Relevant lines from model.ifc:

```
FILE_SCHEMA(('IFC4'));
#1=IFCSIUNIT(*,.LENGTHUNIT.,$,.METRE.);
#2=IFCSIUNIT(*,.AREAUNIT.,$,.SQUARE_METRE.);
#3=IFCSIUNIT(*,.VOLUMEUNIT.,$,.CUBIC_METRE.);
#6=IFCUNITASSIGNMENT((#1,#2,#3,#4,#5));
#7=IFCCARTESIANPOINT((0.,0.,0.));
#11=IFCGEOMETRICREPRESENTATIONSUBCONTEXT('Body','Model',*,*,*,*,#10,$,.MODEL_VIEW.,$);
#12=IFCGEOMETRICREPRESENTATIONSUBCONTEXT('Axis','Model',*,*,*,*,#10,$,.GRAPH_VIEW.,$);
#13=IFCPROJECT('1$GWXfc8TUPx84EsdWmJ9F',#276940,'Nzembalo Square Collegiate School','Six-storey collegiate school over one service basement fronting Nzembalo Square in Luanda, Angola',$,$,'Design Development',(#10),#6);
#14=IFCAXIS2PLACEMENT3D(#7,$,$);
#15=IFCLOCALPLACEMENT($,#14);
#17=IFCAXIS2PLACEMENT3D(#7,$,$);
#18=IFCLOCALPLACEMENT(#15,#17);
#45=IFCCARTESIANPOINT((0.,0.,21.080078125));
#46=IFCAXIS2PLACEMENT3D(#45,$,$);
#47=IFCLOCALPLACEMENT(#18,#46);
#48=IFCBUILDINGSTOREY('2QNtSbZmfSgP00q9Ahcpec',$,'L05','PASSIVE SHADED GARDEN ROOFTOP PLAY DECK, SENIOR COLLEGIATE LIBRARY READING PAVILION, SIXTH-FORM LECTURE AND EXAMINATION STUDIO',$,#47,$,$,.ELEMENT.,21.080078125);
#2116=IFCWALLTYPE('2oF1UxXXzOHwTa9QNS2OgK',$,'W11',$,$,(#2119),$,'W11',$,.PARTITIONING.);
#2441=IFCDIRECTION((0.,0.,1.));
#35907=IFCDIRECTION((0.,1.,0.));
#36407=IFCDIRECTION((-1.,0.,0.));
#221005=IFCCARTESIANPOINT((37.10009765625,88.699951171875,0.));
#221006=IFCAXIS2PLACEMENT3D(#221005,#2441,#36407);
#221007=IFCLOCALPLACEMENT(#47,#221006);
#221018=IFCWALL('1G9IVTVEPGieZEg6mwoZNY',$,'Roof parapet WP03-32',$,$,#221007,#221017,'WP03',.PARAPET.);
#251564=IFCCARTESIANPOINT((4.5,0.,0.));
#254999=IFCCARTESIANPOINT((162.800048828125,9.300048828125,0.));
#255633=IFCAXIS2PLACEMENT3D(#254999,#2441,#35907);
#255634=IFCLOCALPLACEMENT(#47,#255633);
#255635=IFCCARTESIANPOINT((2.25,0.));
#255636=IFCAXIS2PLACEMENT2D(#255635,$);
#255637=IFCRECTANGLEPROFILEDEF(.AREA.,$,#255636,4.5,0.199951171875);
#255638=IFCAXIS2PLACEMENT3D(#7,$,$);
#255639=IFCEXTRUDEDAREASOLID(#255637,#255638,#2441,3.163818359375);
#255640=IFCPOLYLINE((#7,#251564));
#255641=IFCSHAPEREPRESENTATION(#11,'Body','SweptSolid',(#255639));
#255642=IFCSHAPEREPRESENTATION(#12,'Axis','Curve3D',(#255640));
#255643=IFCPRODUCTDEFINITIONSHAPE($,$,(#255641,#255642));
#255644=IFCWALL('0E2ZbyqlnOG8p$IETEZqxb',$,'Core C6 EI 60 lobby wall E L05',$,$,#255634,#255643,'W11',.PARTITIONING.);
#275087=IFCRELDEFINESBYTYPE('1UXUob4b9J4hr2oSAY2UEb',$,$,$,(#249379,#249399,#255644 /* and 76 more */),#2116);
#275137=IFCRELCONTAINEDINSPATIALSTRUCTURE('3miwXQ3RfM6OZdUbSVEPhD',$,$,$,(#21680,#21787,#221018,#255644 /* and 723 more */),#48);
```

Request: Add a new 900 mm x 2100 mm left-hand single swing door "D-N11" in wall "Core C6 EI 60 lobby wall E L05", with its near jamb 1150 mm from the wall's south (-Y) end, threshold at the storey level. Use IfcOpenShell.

```python
import numpy as np
import ifcopenshell
import ifcopenshell.api.feature
import ifcopenshell.api.geometry
import ifcopenshell.api.root
import ifcopenshell.api.spatial
import ifcopenshell.geom
import ifcopenshell.util.element
import ifcopenshell.util.placement
import ifcopenshell.util.representation
import ifcopenshell.util.shape
import ifcopenshell.util.unit

model = ifcopenshell.open("model.ifc")
unit_scale = ifcopenshell.util.unit.calculate_unit_scale(model)
settings = ifcopenshell.geom.settings()


def volume(element):
    """Net volume in cubic metres, openings subtracted."""
    shape = ifcopenshell.geom.create_shape(settings, element)
    return ifcopenshell.util.shape.get_volume(shape.geometry)


wall = model.by_id(255644)
storey = ifcopenshell.util.element.get_container(wall, ifc_class="IfcBuildingStorey")
context = ifcopenshell.util.representation.get_context(model, "Model", "Body", "MODEL_VIEW")
before = volume(wall)

width, height, from_end, sill = 0.9, 2.1, 1.15, 0.0  # metres

# The wall runs along its own X axis, and the end named is its -X end.
wall_shape = ifcopenshell.geom.create_shape(settings, wall)
x, y, z = ifcopenshell.util.shape.get_vertices(wall_shape.geometry).T
start = x.min() + from_end
face, thickness = float(y.min()), float(y.max() - y.min())
wall_matrix = ifcopenshell.util.placement.get_local_placement(wall.ObjectPlacement)
level = ifcopenshell.util.placement.get_local_placement(storey.ObjectPlacement)[2, 3]


def in_wall(x, y):
    """Placement at x, y metres in the wall's axes, at sill height."""
    matrix = wall_matrix.copy()
    matrix[:, 3] = wall_matrix @ np.array([x / unit_scale, y / unit_scale, 0.0, 1.0])
    matrix[2, 3] = level + sill / unit_scale
    return matrix


# Opening: a box that overshoots both wall faces by 50 mm.
opening = ifcopenshell.api.root.create_entity(model, ifc_class="IfcOpeningElement", predefined_type="OPENING")
box = ifcopenshell.api.geometry.add_wall_representation(
    model, context=context, length=width, height=height, thickness=thickness + 0.1
)
ifcopenshell.api.geometry.assign_representation(model, product=opening, representation=box)
ifcopenshell.api.geometry.edit_object_placement(model, product=opening, matrix=in_wall(start, face - 0.05), is_si=False)
ifcopenshell.api.feature.add_feature(model, feature=opening, element=wall)

door = ifcopenshell.api.root.create_entity(model, ifc_class="IfcDoor", name="D-N11", predefined_type="DOOR")
door.OverallWidth, door.OverallHeight = width / unit_scale, height / unit_scale
door.OperationType = "SINGLE_SWING_LEFT"
body = ifcopenshell.api.geometry.add_door_representation(
    model,
    context=context,
    overall_width=door.OverallWidth,
    overall_height=door.OverallHeight,
    operation_type="SINGLE_SWING_LEFT",
    lining_properties={"LiningDepth": thickness / unit_scale, "ThresholdDepth": thickness / unit_scale},
)
ifcopenshell.api.geometry.assign_representation(model, product=door, representation=body)
ifcopenshell.api.spatial.assign_container(model, products=[door], relating_structure=storey)
ifcopenshell.api.feature.add_filling(model, opening=opening, element=door)

# The lining spans the wall, so the door starts at the wall face.
ifcopenshell.api.geometry.edit_object_placement(model, product=door, matrix=in_wall(start, face), is_si=False)

after = volume(wall)

print(f"wall volume {before:.3f} -> {after:.3f} m3")

model.write("model_edited.ifc")
```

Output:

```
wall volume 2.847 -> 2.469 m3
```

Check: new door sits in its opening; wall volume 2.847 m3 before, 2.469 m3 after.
